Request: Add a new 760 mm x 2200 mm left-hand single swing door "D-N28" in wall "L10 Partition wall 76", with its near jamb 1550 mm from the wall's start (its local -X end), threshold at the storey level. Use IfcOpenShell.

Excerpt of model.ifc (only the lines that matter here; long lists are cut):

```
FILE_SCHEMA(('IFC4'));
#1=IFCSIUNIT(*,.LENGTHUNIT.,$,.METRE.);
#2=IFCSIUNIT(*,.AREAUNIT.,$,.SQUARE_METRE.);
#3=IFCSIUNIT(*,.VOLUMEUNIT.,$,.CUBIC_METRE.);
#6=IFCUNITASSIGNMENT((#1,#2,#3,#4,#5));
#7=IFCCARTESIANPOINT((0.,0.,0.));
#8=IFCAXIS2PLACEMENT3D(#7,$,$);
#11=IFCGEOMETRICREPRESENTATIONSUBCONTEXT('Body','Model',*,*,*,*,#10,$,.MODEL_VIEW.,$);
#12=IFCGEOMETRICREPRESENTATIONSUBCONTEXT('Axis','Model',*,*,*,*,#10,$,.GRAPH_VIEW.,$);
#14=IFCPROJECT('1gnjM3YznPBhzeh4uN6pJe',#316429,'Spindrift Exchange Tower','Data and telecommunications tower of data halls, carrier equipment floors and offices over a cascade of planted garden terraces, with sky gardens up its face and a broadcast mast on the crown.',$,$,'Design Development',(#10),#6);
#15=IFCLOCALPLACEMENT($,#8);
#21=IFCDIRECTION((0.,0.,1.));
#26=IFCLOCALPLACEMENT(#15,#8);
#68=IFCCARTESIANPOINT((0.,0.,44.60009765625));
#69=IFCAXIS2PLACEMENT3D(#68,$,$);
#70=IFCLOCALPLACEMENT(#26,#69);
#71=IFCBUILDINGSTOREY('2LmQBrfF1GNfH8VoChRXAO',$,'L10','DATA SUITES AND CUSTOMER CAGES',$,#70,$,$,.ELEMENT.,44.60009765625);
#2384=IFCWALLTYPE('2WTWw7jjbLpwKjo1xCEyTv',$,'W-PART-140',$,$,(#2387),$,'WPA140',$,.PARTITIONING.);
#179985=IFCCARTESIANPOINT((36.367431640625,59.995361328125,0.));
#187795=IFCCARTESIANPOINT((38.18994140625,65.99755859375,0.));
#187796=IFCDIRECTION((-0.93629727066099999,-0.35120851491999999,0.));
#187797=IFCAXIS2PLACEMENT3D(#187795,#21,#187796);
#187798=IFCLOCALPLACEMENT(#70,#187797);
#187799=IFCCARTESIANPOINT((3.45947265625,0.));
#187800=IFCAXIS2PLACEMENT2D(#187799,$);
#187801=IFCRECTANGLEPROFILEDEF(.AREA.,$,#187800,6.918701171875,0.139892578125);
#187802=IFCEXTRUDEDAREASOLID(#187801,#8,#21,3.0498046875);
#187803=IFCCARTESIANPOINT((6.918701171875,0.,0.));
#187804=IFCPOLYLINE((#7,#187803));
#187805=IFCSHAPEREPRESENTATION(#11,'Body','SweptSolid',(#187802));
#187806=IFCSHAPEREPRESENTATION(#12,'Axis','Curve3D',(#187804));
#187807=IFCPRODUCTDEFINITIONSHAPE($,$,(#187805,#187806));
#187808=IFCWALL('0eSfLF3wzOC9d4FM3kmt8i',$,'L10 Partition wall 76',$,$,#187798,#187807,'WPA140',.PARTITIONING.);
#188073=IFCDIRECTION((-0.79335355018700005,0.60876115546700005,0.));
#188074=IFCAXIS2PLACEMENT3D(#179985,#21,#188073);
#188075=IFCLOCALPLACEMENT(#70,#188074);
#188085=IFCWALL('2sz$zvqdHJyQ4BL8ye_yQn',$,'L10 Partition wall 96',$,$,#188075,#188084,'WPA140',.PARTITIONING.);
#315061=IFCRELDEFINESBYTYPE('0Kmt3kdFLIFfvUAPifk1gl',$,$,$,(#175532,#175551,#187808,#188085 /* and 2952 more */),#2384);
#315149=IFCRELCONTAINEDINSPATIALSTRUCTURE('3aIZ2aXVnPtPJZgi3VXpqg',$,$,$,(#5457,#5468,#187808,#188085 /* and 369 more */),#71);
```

```python
import numpy as np
import ifcopenshell
import ifcopenshell.api.feature
import ifcopenshell.api.geometry
import ifcopenshell.api.root
import ifcopenshell.api.spatial
import ifcopenshell.geom
import ifcopenshell.util.element
import ifcopenshell.util.placement
import ifcopenshell.util.representation
import ifcopenshell.util.shape
import ifcopenshell.util.unit

model = ifcopenshell.open("model.ifc")
unit_scale = ifcopenshell.util.unit.calculate_unit_scale(model)
settings = ifcopenshell.geom.settings()


def volume(element):
    """Net volume in cubic metres, openings subtracted."""
    shape = ifcopenshell.geom.create_shape(settings, element)
    return ifcopenshell.util.shape.get_volume(shape.geometry)


wall = model.by_guid("0eSfLF3wzOC9d4FM3kmt8i")
storey = ifcopenshell.util.element.get_container(wall, ifc_class="IfcBuildingStorey")
context = ifcopenshell.util.representation.get_context(model, "Model", "Body", "MODEL_VIEW")
before = volume(wall)

width, height, from_end, sill = 0.76, 2.2, 1.55, 0.0  # metres

# The wall runs along its own X axis, and the end named is its -X end.
wall_shape = ifcopenshell.geom.create_shape(settings, wall)
x, y, z = ifcopenshell.util.shape.get_vertices(wall_shape.geometry).T
start = x.min() + from_end
face, thickness = float(y.min()), float(y.max() - y.min())
wall_matrix = ifcopenshell.util.placement.get_local_placement(wall.ObjectPlacement)
level = ifcopenshell.util.placement.get_local_placement(storey.ObjectPlacement)[2, 3]


def in_wall(x, y):
    """Placement at x, y metres in the wall's axes, at sill height."""
    matrix = wall_matrix.copy()
    matrix[:, 3] = wall_matrix @ np.array([x / unit_scale, y / unit_scale, 0.0, 1.0])
    matrix[2, 3] = level + sill / unit_scale
    return matrix


# Opening: a box that overshoots both wall faces by 50 mm.
opening = ifcopenshell.api.root.create_entity(model, ifc_class="IfcOpeningElement", predefined_type="OPENING")
box = ifcopenshell.api.geometry.add_wall_representation(
    model, context=context, length=width, height=height, thickness=thickness + 0.1
)
ifcopenshell.api.geometry.assign_representation(model, product=opening, representation=box)
ifcopenshell.api.geometry.edit_object_placement(model, product=opening, matrix=in_wall(start, face - 0.05), is_si=False)
ifcopenshell.api.feature.add_feature(model, feature=opening, element=wall)

door = ifcopenshell.api.root.create_entity(model, ifc_class="IfcDoor", name="D-N28", predefined_type="DOOR")
door.OverallWidth, door.OverallHeight = width / unit_scale, height / unit_scale
door.OperationType = "SINGLE_SWING_LEFT"
body = ifcopenshell.api.geometry.add_door_representation(
    model,
    context=context,
    overall_width=door.OverallWidth,
    overall_height=door.OverallHeight,
    operation_type="SINGLE_SWING_LEFT",
    lining_properties={"LiningDepth": thickness / unit_scale, "ThresholdDepth": thickness / unit_scale},
)
ifcopenshell.api.geometry.assign_representation(model, product=door, representation=body)
ifcopenshell.api.spatial.assign_container(model, products=[door], relating_structure=storey)
ifcopenshell.api.feature.add_filling(model, opening=opening, element=door)

# The lining spans the wall, so the door starts at the wall face.
ifcopenshell.api.geometry.edit_object_placement(model, product=door, matrix=in_wall(start, face), is_si=False)

after = volume(wall)

print(f"wall volume {before:.3f} -> {after:.3f} m3")

model.write("model_rev.ifc")
```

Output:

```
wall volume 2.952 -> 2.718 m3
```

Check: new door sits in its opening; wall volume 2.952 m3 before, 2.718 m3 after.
